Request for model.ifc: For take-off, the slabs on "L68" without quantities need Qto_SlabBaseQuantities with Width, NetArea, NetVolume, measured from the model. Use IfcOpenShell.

First a look at what the model holds.

```python
import ifcopenshell
import ifcopenshell.util.element
import ifcopenshell.util.unit

model = ifcopenshell.open("model.ifc")
print(model.schema)
for unit_type in ("LENGTHUNIT", "AREAUNIT", "VOLUMEUNIT"):
    print(unit_type, ifcopenshell.util.unit.calculate_unit_scale(model, unit_type))
storey = next(s for s in model.by_type("IfcBuildingStorey") if s.Name == "L68")
slabs = [e for e in ifcopenshell.util.element.get_decomposition(storey) if e.is_a("IfcSlab")]
for e in sorted(slabs, key=lambda e: e.id()):
    print(e.id(), e.is_a(), e.Name, list(ifcopenshell.util.element.get_psets(e, qtos_only=True)), sep=" | ")
```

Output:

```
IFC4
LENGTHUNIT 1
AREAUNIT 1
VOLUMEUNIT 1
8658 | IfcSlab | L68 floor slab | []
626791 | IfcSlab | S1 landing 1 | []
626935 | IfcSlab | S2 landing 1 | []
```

```python
import ifcopenshell
import ifcopenshell.api.pset
import ifcopenshell.geom
import ifcopenshell.util.element
import ifcopenshell.util.shape
import ifcopenshell.util.unit

model = ifcopenshell.open("model.ifc")
unit_scale = ifcopenshell.util.unit.calculate_unit_scale(model)
area_scale = ifcopenshell.util.unit.calculate_unit_scale(model, "AREAUNIT")
volume_scale = ifcopenshell.util.unit.calculate_unit_scale(model, "VOLUMEUNIT")
settings = ifcopenshell.geom.settings()

storey = next(s for s in model.by_type("IfcBuildingStorey") if s.Name == "L68")
slabs = [e for e in ifcopenshell.util.element.get_decomposition(storey) if e.is_a("IfcSlab")]

for e in sorted(slabs, key=lambda e: e.id()):
    if ifcopenshell.util.element.get_psets(e, qtos_only=True, should_inherit=False):
        continue
    # Geometry comes back in metres, in the element's own axes.
    shape = ifcopenshell.geom.create_shape(settings, e)
    values = {
        "Width": ifcopenshell.util.shape.get_z(shape.geometry) / unit_scale,
        "NetArea": ifcopenshell.util.shape.get_footprint_area(shape.geometry) / area_scale,
        "NetVolume": ifcopenshell.util.shape.get_volume(shape.geometry) / volume_scale,
    }
    qto = ifcopenshell.api.pset.add_qto(model, product=e, name="Qto_SlabBaseQuantities")
    ifcopenshell.api.pset.edit_qto(model, qto=qto, properties=values)
    print(e.id(), {k: round(v, 3) for k, v in values.items()})

model.write("model_updated.ifc")
```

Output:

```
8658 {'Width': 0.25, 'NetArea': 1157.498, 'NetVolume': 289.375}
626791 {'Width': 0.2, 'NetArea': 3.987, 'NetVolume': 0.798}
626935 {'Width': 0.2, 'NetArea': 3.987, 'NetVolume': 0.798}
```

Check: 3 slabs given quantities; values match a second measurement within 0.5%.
